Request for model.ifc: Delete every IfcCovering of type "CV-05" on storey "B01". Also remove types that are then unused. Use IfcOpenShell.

First a look at what the model holds.

```python
import ifcopenshell
import ifcopenshell.util.element

model = ifcopenshell.open("model.ifc")
print(model.schema)
storey = next(s for s in model.by_type("IfcBuildingStorey") if s.Name == "B01")
coverings = [e for e in ifcopenshell.util.element.get_decomposition(storey) if e.is_a("IfcCovering")]
seen = {}
for e in coverings:
    element_type = ifcopenshell.util.element.get_type(e)
    name = element_type.Name if element_type not in (None, e) else None
    seen[name] = seen.get(name, 0) + 1
for name, count in sorted(seen.items(), key=str):
    print(count, "x", name)
```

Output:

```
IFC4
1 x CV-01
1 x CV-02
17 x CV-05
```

```python
import ifcopenshell
import ifcopenshell.api.root
import ifcopenshell.util.element

model = ifcopenshell.open("model.ifc")

storey = next(s for s in model.by_type("IfcBuildingStorey") if s.Name == "B01")
coverings = [e for e in ifcopenshell.util.element.get_decomposition(storey) if e.is_a("IfcCovering")]
targets = [e for e in coverings if (t := ifcopenshell.util.element.get_type(e)) not in (None, e) and t.Name == "CV-05"]
types = {ifcopenshell.util.element.get_type(e) for e in targets} - {None, *targets}

for e in targets:
    ifcopenshell.api.root.remove_product(model, product=e)
print(len(targets), "removed")

unused = [t for t in types if not ifcopenshell.util.element.get_types(t)]
for t in unused:
    ifcopenshell.api.root.remove_product(model, product=t)
print(len(unused), "unused types removed")

model.write("model_edited.ifc")
```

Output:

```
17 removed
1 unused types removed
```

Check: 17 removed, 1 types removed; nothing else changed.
